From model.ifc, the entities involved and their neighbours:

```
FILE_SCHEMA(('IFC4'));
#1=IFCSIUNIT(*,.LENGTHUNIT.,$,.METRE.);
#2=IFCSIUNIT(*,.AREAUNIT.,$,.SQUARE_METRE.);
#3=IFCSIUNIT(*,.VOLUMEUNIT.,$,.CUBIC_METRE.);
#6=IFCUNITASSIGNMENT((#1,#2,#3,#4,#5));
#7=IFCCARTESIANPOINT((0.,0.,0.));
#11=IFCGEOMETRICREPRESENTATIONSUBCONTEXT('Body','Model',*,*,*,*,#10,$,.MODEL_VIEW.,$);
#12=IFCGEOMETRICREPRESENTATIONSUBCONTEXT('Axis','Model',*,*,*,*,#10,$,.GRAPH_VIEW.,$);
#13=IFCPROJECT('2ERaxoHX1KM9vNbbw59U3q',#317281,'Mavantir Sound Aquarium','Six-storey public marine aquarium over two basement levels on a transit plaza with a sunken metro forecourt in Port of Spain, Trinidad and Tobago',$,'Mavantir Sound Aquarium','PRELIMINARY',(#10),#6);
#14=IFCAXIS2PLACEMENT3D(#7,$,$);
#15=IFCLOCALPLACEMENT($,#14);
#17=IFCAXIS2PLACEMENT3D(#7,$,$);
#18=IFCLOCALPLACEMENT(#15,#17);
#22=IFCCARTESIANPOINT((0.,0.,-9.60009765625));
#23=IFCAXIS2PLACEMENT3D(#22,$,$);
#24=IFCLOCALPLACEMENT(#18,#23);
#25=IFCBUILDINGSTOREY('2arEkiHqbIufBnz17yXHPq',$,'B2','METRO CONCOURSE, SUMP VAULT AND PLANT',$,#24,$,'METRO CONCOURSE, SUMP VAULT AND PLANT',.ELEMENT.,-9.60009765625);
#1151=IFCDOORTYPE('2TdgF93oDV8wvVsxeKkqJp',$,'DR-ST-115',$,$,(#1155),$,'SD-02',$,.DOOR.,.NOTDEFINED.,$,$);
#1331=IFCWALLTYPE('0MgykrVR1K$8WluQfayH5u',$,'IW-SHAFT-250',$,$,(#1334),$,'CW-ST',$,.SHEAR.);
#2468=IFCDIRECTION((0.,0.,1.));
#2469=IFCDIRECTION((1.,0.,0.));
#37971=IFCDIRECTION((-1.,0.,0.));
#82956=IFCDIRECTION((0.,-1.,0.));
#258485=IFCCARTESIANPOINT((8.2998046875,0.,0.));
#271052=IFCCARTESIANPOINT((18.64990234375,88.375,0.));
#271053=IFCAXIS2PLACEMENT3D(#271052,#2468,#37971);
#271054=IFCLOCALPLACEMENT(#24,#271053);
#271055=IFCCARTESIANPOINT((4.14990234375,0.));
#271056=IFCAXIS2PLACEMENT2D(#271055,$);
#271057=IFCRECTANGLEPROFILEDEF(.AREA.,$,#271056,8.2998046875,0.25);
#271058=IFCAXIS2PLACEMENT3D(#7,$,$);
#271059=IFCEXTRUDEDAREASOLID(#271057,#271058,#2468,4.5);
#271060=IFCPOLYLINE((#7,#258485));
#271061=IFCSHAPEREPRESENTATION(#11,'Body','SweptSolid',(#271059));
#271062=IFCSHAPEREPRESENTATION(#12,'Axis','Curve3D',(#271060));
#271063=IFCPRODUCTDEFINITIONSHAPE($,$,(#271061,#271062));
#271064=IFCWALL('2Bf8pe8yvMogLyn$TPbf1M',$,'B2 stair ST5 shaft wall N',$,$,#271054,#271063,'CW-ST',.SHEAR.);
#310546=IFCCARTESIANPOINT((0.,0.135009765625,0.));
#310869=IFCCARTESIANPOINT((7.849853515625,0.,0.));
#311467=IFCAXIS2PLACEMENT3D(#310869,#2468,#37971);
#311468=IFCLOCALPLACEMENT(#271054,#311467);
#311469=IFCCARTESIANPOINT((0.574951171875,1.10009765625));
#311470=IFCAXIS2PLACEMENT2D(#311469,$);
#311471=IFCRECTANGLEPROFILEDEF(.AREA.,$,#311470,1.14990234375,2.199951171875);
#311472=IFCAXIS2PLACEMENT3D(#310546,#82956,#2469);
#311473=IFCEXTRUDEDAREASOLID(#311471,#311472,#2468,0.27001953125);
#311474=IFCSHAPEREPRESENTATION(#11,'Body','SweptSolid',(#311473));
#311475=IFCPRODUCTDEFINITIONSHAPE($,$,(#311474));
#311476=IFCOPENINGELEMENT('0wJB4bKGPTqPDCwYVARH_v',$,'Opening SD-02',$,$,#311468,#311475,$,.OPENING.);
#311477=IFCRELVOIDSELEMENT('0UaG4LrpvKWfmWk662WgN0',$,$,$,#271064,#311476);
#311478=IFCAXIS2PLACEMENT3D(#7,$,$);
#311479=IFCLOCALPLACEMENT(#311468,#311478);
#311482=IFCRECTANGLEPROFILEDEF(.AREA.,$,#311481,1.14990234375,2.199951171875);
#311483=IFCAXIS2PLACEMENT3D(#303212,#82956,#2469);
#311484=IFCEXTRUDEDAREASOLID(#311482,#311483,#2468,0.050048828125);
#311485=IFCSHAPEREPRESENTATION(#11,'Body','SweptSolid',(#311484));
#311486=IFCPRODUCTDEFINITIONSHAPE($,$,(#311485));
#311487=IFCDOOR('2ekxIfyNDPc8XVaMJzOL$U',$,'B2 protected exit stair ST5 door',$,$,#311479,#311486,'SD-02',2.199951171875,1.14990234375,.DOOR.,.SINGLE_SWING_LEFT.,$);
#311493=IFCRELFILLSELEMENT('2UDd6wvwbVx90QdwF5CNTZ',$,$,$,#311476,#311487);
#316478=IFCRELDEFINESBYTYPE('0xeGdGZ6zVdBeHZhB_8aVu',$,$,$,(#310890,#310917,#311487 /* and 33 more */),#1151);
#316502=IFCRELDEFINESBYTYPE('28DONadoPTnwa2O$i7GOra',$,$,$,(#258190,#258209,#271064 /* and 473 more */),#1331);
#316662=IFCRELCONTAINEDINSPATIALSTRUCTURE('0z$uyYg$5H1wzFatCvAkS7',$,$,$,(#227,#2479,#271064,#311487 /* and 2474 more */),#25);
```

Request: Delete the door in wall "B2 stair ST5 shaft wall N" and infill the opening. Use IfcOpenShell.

```python
import ifcopenshell
import ifcopenshell.api.feature
import ifcopenshell.api.root
import ifcopenshell.geom
import ifcopenshell.util.shape

model = ifcopenshell.open("model.ifc")
settings = ifcopenshell.geom.settings()


def volume(element):
    """Net volume in cubic metres, openings subtracted."""
    shape = ifcopenshell.geom.create_shape(settings, element)
    return ifcopenshell.util.shape.get_volume(shape.geometry)


door = model.by_guid("2ekxIfyNDPc8XVaMJzOL$U")
opening = door.FillsVoids[0].RelatingOpeningElement
wall = opening.VoidsElements[0].RelatingBuildingElement
before = volume(wall)

ifcopenshell.api.root.remove_product(model, product=door)
ifcopenshell.api.feature.remove_feature(model, feature=opening)

after = volume(wall)

print(f"wall volume {before:.3f} -> {after:.3f} m3")

model.write("model_edited.ifc")
```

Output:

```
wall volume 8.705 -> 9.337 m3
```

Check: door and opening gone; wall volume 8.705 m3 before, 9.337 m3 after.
